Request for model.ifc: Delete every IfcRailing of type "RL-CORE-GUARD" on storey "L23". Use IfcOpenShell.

First a look at what the model holds.

```python
import ifcopenshell
import ifcopenshell.util.element

model = ifcopenshell.open("model.ifc")
print(model.schema)
storey = next(s for s in model.by_type("IfcBuildingStorey") if s.Name == "L23")
railings = [e for e in ifcopenshell.util.element.get_decomposition(storey) if e.is_a("IfcRailing")]
seen = {}
for e in railings:
    element_type = ifcopenshell.util.element.get_type(e)
    name = element_type.Name if element_type not in (None, e) else None
    seen[name] = seen.get(name, 0) + 1
for name, count in sorted(seen.items(), key=str):
    print(count, "x", name)
```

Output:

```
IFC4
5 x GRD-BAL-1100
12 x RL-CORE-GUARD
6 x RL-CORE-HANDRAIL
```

```python
import ifcopenshell
import ifcopenshell.api.root
import ifcopenshell.util.element

model = ifcopenshell.open("model.ifc")

storey = next(s for s in model.by_type("IfcBuildingStorey") if s.Name == "L23")
railings = [e for e in ifcopenshell.util.element.get_decomposition(storey) if e.is_a("IfcRailing")]
targets = [e for e in railings if (t := ifcopenshell.util.element.get_type(e)) not in (None, e) and t.Name == "RL-CORE-GUARD"]

for e in targets:
    ifcopenshell.api.root.remove_product(model, product=e)
print(len(targets), "removed")

model.write("model-out.ifc")
```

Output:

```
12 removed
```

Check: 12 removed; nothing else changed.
